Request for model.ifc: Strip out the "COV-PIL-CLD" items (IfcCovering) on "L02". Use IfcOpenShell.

First a look at what the model holds.

```python
import ifcopenshell
import ifcopenshell.util.element

model = ifcopenshell.open("model.ifc")
print(model.schema)
storey = next(s for s in model.by_type("IfcBuildingStorey") if s.Name == "L02")
coverings = [e for e in ifcopenshell.util.element.get_decomposition(storey) if e.is_a("IfcCovering")]
seen = {}
for e in coverings:
    element_type = ifcopenshell.util.element.get_type(e)
    name = element_type.Name if element_type not in (None, e) else None
    seen[name] = seen.get(name, 0) + 1
for name, count in sorted(seen.items(), key=str):
    print(count, "x", name)
```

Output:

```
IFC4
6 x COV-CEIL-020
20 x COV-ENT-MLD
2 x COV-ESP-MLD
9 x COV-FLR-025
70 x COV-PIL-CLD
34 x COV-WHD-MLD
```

```python
import ifcopenshell
import ifcopenshell.api.root
import ifcopenshell.util.element

model = ifcopenshell.open("model.ifc")

storey = next(s for s in model.by_type("IfcBuildingStorey") if s.Name == "L02")
coverings = [e for e in ifcopenshell.util.element.get_decomposition(storey) if e.is_a("IfcCovering")]
targets = [e for e in coverings if (t := ifcopenshell.util.element.get_type(e)) not in (None, e) and t.Name == "COV-PIL-CLD"]

for e in targets:
    ifcopenshell.api.root.remove_product(model, product=e)
print(len(targets), "removed")

model.write("model_edited.ifc")
```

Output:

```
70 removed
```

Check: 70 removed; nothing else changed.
